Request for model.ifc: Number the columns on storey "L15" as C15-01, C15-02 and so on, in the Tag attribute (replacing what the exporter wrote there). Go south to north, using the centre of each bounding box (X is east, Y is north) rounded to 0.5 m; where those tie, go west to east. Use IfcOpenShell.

First a look at what the model holds.

```python
import ifcopenshell
import ifcopenshell.util.element
import ifcopenshell.util.placement

model = ifcopenshell.open("model.ifc")
print(model.schema)
storey = next(s for s in model.by_type("IfcBuildingStorey") if s.Name == "L15")
columns = [e for e in ifcopenshell.util.element.get_decomposition(storey) if e.is_a("IfcColumn")]
for e in sorted(columns, key=lambda e: e.id()):
    origin = ifcopenshell.util.placement.get_local_placement(e.ObjectPlacement)[:3, 3]
    print(e.id(), e.Tag, e.Name, origin.round(2) + 0.0, sep=" | ")
```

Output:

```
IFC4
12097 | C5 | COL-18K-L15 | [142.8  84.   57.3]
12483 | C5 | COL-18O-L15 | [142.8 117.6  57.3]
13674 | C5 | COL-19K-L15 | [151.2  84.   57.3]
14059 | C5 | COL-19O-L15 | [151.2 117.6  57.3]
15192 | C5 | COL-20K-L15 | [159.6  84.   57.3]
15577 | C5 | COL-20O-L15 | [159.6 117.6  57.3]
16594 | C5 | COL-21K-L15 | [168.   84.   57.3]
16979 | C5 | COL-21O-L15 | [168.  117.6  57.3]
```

```python
import ifcopenshell
import ifcopenshell.geom
import ifcopenshell.util.element
import ifcopenshell.util.shape

model = ifcopenshell.open("model.ifc")
settings = ifcopenshell.geom.settings()
settings.set("use-world-coords", True)


def centre(element):
    shape = ifcopenshell.geom.create_shape(settings, element)
    return ifcopenshell.util.shape.get_bbox_centroid(shape.geometry)


storey = next(s for s in model.by_type("IfcBuildingStorey") if s.Name == "L15")
columns = [e for e in ifcopenshell.util.element.get_decomposition(storey) if e.is_a("IfcColumn")]

# Insertion points can sit at a corner or the storey origin, so sort by the geometry (in metres).
centres = {e: centre(e) for e in columns}
columns.sort(key=lambda e: (round(centres[e][1] / 0.5), centres[e][0]))

for i, e in enumerate(columns, start=1):
    number = f"C15-{i:02d}"
    e.Tag = number
    print(e.id(), number)

model.write("model_edited.ifc")
```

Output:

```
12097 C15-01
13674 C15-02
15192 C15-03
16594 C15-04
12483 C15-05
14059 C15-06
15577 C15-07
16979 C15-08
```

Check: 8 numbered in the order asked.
